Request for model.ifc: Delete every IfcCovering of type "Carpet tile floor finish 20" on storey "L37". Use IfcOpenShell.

First a look at what the model holds.

```python
import ifcopenshell
import ifcopenshell.util.element

model = ifcopenshell.open("model.ifc")
print(model.schema)
storey = next(s for s in model.by_type("IfcBuildingStorey") if s.Name == "L37")
coverings = [e for e in ifcopenshell.util.element.get_decomposition(storey) if e.is_a("IfcCovering")]
seen = {}
for e in coverings:
    element_type = ifcopenshell.util.element.get_type(e)
    name = element_type.Name if element_type not in (None, e) else None
    seen[name] = seen.get(name, 0) + 1
for name, count in sorted(seen.items(), key=str):
    print(count, "x", name)
```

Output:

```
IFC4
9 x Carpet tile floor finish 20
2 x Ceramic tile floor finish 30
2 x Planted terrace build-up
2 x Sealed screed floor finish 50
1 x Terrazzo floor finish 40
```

```python
import ifcopenshell
import ifcopenshell.api.root
import ifcopenshell.util.element

model = ifcopenshell.open("model.ifc")

storey = next(s for s in model.by_type("IfcBuildingStorey") if s.Name == "L37")
coverings = [e for e in ifcopenshell.util.element.get_decomposition(storey) if e.is_a("IfcCovering")]
targets = [e for e in coverings if (t := ifcopenshell.util.element.get_type(e)) not in (None, e) and t.Name == "Carpet tile floor finish 20"]

for e in targets:
    ifcopenshell.api.root.remove_product(model, product=e)
print(len(targets), "removed")

model.write("model_rev.ifc")
```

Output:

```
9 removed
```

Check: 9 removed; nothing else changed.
